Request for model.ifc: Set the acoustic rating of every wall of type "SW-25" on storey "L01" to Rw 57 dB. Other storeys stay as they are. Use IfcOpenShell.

First a look at what the model holds.

```python
import ifcopenshell
import ifcopenshell.util.element

model = ifcopenshell.open("model.ifc")
print(model.schema)
storey = next(s for s in model.by_type("IfcBuildingStorey") if s.Name == "L01")
walls = [e for e in ifcopenshell.util.element.get_decomposition(storey) if e.is_a("IfcWall")]
seen = {}
for e in walls:
    element_type = ifcopenshell.util.element.get_type(e)
    key = (element_type.Name if element_type != e and element_type else None, ifcopenshell.util.element.get_pset(e, "Pset_WallCommon", "AcousticRating"))
    seen[key] = seen.get(key, 0) + 1
for (name, value), count in sorted(seen.items(), key=str):
    print(count, "x", name, "|", value)
```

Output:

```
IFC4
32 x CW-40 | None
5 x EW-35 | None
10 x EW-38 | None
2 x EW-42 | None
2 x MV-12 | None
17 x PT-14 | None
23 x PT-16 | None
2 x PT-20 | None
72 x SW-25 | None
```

```python
import ifcopenshell
import ifcopenshell.api.pset
import ifcopenshell.util.element

model = ifcopenshell.open("model.ifc")

storey = next(s for s in model.by_type("IfcBuildingStorey") if s.Name == "L01")
walls = [e for e in ifcopenshell.util.element.get_decomposition(storey) if e.is_a("IfcWall")]

count = 0
for e in walls:
    element_type = ifcopenshell.util.element.get_type(e)
    if element_type in (None, e) or element_type.Name != "SW-25":
        continue
    # add_pset returns the element's existing set when there is one.
    pset = ifcopenshell.api.pset.add_pset(model, product=e, name="Pset_WallCommon")
    ifcopenshell.api.pset.edit_pset(model, pset=pset, properties={"AcousticRating": "Rw 57 dB"})
    count += 1

print(count, "walls updated")

model.write("model_v2.ifc")
```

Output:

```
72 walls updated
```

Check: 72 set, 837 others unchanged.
